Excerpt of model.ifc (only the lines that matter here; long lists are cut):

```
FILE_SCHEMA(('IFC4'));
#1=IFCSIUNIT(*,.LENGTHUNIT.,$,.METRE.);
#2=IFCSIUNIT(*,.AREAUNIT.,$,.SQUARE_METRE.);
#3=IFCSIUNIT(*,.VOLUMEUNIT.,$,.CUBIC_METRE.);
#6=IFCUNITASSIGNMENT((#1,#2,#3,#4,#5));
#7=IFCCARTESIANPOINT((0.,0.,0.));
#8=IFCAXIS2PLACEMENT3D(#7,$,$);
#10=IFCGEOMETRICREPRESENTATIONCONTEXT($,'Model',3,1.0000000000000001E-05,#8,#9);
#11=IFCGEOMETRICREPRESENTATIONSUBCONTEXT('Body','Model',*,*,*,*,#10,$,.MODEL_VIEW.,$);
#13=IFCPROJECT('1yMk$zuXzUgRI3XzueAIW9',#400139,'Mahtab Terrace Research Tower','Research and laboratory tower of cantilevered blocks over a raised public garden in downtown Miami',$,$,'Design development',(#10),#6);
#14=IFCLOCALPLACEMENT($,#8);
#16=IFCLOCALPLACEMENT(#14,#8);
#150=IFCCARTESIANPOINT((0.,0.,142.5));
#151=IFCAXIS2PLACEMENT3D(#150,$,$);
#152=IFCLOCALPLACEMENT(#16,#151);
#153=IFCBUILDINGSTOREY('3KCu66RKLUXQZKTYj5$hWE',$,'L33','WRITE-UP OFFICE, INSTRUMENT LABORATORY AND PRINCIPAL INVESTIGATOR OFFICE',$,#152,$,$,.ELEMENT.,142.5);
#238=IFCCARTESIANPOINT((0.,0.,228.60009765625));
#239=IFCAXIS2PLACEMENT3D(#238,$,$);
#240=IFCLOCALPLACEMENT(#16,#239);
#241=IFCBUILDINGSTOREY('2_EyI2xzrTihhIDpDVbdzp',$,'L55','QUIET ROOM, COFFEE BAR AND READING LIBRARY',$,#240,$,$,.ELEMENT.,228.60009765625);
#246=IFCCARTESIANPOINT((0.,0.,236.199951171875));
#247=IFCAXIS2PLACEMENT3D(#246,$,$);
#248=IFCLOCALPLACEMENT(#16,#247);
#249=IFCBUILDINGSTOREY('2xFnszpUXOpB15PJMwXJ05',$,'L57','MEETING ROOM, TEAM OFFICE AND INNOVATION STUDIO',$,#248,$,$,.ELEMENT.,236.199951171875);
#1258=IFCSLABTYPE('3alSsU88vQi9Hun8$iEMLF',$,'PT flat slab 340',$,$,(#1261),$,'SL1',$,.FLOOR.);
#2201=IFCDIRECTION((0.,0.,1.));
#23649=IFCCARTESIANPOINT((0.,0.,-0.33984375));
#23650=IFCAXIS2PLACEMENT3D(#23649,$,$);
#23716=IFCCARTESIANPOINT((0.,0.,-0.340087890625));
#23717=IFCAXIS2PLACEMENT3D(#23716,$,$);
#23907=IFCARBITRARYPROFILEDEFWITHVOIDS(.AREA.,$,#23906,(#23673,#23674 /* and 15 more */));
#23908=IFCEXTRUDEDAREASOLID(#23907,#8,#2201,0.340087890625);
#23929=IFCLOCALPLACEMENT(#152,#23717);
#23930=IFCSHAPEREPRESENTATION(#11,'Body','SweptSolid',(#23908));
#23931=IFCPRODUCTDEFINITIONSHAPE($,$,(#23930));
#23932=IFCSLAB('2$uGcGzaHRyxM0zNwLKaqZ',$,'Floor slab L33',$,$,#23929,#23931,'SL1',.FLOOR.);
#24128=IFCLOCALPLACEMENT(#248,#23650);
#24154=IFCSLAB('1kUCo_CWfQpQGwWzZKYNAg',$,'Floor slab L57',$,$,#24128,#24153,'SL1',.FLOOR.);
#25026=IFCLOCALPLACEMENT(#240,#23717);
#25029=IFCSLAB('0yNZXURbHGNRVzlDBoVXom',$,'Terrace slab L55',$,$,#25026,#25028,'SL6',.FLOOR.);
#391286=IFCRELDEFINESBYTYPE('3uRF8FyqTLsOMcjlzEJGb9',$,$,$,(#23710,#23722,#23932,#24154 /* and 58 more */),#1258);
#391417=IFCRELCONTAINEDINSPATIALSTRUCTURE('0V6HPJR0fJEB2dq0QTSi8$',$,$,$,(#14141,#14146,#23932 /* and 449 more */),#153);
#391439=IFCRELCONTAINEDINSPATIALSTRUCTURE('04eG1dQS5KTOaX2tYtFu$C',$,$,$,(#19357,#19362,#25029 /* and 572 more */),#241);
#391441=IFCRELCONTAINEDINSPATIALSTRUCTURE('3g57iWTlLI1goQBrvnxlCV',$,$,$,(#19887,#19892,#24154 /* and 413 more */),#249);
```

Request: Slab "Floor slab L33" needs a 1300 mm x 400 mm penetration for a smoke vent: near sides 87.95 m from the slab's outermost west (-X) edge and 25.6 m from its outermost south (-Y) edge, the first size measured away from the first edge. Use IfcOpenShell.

```python
import numpy as np
import ifcopenshell
import ifcopenshell.api.feature
import ifcopenshell.api.geometry
import ifcopenshell.api.root
import ifcopenshell.geom
import ifcopenshell.util.placement
import ifcopenshell.util.representation
import ifcopenshell.util.shape
import ifcopenshell.util.unit

model = ifcopenshell.open("model.ifc")
unit_scale = ifcopenshell.util.unit.calculate_unit_scale(model)
settings = ifcopenshell.geom.settings()


def volume(element):
    """Net volume in cubic metres, openings subtracted."""
    shape = ifcopenshell.geom.create_shape(settings, element)
    return ifcopenshell.util.shape.get_volume(shape.geometry)


slab = model.by_guid("2$uGcGzaHRyxM0zNwLKaqZ")
before = volume(slab)

# Extent in the slab's own axes, in metres. The edges named are its -X and -Y sides.
slab_shape = ifcopenshell.geom.create_shape(settings, slab)
vertices = ifcopenshell.util.shape.get_vertices(slab_shape.geometry)
x_min, y_min, bottom = vertices.min(axis=0)
top = vertices[:, 2].max()

opening = ifcopenshell.api.root.create_entity(model, ifc_class="IfcOpeningElement", name="Smoke vent opening", predefined_type="OPENING")
context = ifcopenshell.util.representation.get_context(model, "Model", "Body", "MODEL_VIEW")
width, depth = 1.3, 0.4
outline = [(0.0, 0.0), (width, 0.0), (width, depth), (0.0, depth), (0.0, 0.0)]
# Overshoot both faces by 50 mm so the cut is clean.
shape = ifcopenshell.api.geometry.add_slab_representation(
    model, context=context, depth=top - bottom + 0.1, polyline=outline
)
ifcopenshell.api.geometry.assign_representation(model, product=opening, representation=shape)

matrix = ifcopenshell.util.placement.get_local_placement(slab.ObjectPlacement)
matrix[:, 3] = matrix @ np.append(np.array([x_min + 87.95, y_min + 25.6, bottom - 0.05]) / unit_scale, 1.0)
ifcopenshell.api.geometry.edit_object_placement(model, product=opening, matrix=matrix, is_si=False)
ifcopenshell.api.feature.add_feature(model, feature=opening, element=slab)

after = volume(slab)

print(f"slab volume {before:.3f} -> {after:.3f} m3")

model.write("model_v2.ifc")
```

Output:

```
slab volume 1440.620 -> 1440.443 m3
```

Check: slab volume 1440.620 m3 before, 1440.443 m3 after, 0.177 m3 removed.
